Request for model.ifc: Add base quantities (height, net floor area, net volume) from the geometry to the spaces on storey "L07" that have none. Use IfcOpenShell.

First a look at what the model holds.

```python
import ifcopenshell
import ifcopenshell.util.element
import ifcopenshell.util.unit

model = ifcopenshell.open("model.ifc")
print(model.schema)
for unit_type in ("LENGTHUNIT", "AREAUNIT", "VOLUMEUNIT"):
    print(unit_type, ifcopenshell.util.unit.calculate_unit_scale(model, unit_type))
storey = next(s for s in model.by_type("IfcBuildingStorey") if s.Name == "L07")
spaces = [e for e in ifcopenshell.util.element.get_decomposition(storey) if e.is_a("IfcSpace")]
for e in sorted(spaces, key=lambda e: e.id()):
    print(e.id(), e.is_a(), e.Name, list(ifcopenshell.util.element.get_psets(e, qtos_only=True)), sep=" | ")
```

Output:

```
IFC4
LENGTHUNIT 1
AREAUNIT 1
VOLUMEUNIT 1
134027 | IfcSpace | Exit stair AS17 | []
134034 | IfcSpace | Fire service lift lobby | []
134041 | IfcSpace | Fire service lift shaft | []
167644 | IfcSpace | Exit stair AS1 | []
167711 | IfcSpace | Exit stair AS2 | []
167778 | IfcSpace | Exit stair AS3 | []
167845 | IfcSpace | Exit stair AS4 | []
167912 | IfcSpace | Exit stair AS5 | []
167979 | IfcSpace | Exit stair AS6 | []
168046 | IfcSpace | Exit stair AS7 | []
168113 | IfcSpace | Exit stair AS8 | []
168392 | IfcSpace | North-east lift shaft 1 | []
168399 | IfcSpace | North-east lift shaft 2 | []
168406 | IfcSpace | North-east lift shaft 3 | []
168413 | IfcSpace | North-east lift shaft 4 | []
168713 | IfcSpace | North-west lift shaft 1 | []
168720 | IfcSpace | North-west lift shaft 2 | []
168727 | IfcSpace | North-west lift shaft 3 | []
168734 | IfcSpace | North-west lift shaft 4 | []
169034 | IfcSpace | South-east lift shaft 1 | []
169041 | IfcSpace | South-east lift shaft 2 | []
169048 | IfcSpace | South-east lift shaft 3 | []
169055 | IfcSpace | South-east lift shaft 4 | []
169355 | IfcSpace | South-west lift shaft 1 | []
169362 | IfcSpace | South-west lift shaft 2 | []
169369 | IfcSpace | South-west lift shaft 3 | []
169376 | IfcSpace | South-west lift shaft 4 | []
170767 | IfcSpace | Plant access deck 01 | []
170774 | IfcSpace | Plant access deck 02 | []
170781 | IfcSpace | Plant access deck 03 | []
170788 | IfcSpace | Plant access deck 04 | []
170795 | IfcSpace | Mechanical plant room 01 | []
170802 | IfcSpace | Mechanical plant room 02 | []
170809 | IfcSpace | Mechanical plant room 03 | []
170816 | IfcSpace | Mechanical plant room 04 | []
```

```python
import ifcopenshell
import ifcopenshell.api.pset
import ifcopenshell.geom
import ifcopenshell.util.element
import ifcopenshell.util.shape
import ifcopenshell.util.unit

model = ifcopenshell.open("model.ifc")
unit_scale = ifcopenshell.util.unit.calculate_unit_scale(model)
area_scale = ifcopenshell.util.unit.calculate_unit_scale(model, "AREAUNIT")
volume_scale = ifcopenshell.util.unit.calculate_unit_scale(model, "VOLUMEUNIT")
settings = ifcopenshell.geom.settings()

storey = next(s for s in model.by_type("IfcBuildingStorey") if s.Name == "L07")
spaces = [e for e in ifcopenshell.util.element.get_decomposition(storey) if e.is_a("IfcSpace")]

for e in sorted(spaces, key=lambda e: e.id()):
    if ifcopenshell.util.element.get_psets(e, qtos_only=True, should_inherit=False):
        continue
    # Geometry comes back in metres, in the element's own axes.
    shape = ifcopenshell.geom.create_shape(settings, e)
    values = {
        "Height": ifcopenshell.util.shape.get_z(shape.geometry) / unit_scale,
        "NetFloorArea": ifcopenshell.util.shape.get_footprint_area(shape.geometry) / area_scale,
        "NetVolume": ifcopenshell.util.shape.get_volume(shape.geometry) / volume_scale,
    }
    qto = ifcopenshell.api.pset.add_qto(model, product=e, name="Qto_SpaceBaseQuantities")
    ifcopenshell.api.pset.edit_qto(model, qto=qto, properties=values)
    print(e.id(), {k: round(v, 3) for k, v in values.items()})

model.write("model_rev.ifc")
```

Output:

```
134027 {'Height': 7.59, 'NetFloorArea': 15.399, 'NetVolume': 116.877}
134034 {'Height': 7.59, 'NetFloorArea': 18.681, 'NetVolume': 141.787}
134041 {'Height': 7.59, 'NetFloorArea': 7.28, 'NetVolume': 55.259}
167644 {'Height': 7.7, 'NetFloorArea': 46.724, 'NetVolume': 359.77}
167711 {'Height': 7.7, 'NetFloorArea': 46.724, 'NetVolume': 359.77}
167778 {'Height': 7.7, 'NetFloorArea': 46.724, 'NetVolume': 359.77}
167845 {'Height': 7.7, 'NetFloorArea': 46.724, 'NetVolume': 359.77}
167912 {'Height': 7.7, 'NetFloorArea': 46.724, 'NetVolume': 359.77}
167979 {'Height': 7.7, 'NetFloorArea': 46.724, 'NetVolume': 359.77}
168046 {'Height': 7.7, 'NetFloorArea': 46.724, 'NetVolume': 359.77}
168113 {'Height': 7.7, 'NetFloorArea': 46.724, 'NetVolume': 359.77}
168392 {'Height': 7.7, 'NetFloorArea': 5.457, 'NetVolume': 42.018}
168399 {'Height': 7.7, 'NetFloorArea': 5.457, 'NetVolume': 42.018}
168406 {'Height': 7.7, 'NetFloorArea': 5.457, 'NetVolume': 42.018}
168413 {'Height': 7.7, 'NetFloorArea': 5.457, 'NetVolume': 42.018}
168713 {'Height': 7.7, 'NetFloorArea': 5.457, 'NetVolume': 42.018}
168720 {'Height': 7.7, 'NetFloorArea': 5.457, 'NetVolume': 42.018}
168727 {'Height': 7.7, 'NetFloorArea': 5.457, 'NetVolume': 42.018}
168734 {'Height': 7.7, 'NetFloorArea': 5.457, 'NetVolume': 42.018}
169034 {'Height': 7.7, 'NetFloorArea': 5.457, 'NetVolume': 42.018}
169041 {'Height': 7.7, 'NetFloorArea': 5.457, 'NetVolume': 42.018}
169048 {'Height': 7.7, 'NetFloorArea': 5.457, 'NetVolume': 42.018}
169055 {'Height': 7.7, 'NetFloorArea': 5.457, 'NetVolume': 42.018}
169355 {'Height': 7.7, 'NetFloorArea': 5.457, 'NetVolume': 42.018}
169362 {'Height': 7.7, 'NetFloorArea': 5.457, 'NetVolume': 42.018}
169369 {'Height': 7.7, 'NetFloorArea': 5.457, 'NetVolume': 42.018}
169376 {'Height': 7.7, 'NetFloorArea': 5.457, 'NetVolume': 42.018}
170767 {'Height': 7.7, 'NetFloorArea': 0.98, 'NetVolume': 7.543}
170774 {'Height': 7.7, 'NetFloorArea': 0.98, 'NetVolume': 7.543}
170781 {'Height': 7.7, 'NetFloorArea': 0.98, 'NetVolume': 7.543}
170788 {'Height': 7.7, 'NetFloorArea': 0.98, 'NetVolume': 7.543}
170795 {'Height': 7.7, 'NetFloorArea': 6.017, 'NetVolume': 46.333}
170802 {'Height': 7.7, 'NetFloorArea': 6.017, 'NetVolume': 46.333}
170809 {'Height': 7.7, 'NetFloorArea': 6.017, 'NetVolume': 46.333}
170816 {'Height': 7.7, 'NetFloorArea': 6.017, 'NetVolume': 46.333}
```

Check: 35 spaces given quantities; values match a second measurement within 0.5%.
